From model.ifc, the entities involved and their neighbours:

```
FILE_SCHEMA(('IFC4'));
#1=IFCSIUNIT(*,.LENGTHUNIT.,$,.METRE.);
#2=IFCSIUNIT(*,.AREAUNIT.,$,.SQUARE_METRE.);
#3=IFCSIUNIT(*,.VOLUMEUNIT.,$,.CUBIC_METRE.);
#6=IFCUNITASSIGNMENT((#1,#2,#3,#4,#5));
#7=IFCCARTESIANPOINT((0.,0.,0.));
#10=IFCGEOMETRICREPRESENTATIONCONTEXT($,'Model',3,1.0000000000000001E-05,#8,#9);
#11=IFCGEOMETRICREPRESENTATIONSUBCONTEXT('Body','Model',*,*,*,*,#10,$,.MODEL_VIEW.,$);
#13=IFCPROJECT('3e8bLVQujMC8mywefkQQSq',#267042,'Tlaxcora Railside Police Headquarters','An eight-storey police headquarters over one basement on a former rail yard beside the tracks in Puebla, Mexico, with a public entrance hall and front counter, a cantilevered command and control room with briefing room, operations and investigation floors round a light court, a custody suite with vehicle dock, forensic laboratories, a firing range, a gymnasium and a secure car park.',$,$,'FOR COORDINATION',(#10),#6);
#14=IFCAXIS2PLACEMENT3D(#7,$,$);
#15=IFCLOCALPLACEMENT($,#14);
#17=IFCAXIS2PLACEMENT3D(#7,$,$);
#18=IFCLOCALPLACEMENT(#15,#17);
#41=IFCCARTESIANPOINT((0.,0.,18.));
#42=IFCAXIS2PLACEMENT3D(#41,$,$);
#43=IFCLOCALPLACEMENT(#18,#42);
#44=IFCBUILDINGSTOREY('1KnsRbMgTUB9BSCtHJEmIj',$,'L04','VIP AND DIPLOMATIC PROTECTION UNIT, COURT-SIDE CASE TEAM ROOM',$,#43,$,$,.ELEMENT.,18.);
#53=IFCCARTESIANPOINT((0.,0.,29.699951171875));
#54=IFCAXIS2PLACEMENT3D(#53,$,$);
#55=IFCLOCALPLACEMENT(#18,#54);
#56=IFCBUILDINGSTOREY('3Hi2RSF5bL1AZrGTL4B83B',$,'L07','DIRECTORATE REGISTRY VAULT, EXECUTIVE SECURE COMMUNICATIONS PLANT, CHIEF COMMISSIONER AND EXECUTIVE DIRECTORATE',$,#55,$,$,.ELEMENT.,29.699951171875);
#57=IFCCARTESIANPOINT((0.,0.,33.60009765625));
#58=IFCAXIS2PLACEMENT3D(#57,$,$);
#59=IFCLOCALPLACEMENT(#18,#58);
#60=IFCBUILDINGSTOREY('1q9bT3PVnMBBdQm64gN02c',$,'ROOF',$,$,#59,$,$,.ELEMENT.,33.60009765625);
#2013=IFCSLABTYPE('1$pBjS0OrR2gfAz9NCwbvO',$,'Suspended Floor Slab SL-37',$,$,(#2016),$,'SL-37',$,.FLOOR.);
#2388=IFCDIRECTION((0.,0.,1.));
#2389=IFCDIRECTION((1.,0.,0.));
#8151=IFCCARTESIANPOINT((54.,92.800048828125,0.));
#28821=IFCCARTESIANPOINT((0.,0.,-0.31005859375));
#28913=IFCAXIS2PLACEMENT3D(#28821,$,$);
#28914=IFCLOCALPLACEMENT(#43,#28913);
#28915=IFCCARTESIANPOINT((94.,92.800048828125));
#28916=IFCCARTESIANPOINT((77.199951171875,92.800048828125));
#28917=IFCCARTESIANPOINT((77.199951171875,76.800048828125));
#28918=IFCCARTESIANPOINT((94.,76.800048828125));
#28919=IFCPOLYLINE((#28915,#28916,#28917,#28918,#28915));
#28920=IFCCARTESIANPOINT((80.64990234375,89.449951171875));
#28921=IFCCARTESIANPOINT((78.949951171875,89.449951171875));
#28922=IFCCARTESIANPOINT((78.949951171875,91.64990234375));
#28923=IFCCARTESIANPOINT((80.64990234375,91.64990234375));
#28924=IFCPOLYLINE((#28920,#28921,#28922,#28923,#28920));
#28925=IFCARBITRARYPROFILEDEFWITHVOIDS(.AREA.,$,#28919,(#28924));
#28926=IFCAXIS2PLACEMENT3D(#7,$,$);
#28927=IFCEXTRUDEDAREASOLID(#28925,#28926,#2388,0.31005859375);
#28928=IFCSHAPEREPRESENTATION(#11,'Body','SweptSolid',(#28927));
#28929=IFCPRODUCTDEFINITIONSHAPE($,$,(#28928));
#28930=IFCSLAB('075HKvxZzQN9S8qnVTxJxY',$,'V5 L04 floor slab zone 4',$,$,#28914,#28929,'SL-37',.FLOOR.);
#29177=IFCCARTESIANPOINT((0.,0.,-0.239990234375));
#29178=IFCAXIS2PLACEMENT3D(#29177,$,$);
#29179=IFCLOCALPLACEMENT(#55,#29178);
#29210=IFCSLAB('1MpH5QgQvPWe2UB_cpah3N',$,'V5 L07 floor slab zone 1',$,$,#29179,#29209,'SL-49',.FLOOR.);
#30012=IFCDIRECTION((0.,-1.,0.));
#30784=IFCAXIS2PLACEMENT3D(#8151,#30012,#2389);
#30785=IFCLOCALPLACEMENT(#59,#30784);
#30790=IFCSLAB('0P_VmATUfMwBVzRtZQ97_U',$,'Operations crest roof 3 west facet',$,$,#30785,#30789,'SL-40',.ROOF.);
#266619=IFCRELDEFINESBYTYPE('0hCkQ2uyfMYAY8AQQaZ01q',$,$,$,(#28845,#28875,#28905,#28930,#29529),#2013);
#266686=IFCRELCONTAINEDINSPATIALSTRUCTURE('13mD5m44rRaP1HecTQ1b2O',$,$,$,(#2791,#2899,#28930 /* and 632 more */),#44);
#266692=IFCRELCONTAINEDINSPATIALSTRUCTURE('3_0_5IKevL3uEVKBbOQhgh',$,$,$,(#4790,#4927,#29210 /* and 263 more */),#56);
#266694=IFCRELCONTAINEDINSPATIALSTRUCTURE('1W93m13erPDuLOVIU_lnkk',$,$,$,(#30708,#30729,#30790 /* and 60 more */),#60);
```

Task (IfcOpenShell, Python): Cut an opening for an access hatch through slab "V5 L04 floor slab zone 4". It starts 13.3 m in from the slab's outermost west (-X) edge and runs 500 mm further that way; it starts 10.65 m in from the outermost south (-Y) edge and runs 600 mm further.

```python
import numpy as np
import ifcopenshell
import ifcopenshell.api.feature
import ifcopenshell.api.geometry
import ifcopenshell.api.root
import ifcopenshell.geom
import ifcopenshell.util.placement
import ifcopenshell.util.representation
import ifcopenshell.util.shape
import ifcopenshell.util.unit

model = ifcopenshell.open("model.ifc")
unit_scale = ifcopenshell.util.unit.calculate_unit_scale(model)
settings = ifcopenshell.geom.settings()


def volume(element):
    """Net volume in cubic metres, openings subtracted."""
    shape = ifcopenshell.geom.create_shape(settings, element)
    return ifcopenshell.util.shape.get_volume(shape.geometry)


slab = model.by_guid("075HKvxZzQN9S8qnVTxJxY")
before = volume(slab)

# Extent in the slab's own axes, in metres. The edges named are its -X and -Y sides.
slab_shape = ifcopenshell.geom.create_shape(settings, slab)
vertices = ifcopenshell.util.shape.get_vertices(slab_shape.geometry)
x_min, y_min, bottom = vertices.min(axis=0)
top = vertices[:, 2].max()

opening = ifcopenshell.api.root.create_entity(model, ifc_class="IfcOpeningElement", name="Access hatch opening", predefined_type="OPENING")
context = ifcopenshell.util.representation.get_context(model, "Model", "Body", "MODEL_VIEW")
width, depth = 0.5, 0.6
outline = [(0.0, 0.0), (width, 0.0), (width, depth), (0.0, depth), (0.0, 0.0)]
# Overshoot both faces by 50 mm so the cut is clean.
shape = ifcopenshell.api.geometry.add_slab_representation(
    model, context=context, depth=top - bottom + 0.1, polyline=outline
)
ifcopenshell.api.geometry.assign_representation(model, product=opening, representation=shape)

matrix = ifcopenshell.util.placement.get_local_placement(slab.ObjectPlacement)
matrix[:, 3] = matrix @ np.append(np.array([x_min + 13.3, y_min + 10.65, bottom - 0.05]) / unit_scale, 1.0)
ifcopenshell.api.geometry.edit_object_placement(model, product=opening, matrix=matrix, is_si=False)
ifcopenshell.api.feature.add_feature(model, feature=opening, element=slab)

after = volume(slab)

print(f"slab volume {before:.3f} -> {after:.3f} m3")

model.write("model_updated.ifc")
```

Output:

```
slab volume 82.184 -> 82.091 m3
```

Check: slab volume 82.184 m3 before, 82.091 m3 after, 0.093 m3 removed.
